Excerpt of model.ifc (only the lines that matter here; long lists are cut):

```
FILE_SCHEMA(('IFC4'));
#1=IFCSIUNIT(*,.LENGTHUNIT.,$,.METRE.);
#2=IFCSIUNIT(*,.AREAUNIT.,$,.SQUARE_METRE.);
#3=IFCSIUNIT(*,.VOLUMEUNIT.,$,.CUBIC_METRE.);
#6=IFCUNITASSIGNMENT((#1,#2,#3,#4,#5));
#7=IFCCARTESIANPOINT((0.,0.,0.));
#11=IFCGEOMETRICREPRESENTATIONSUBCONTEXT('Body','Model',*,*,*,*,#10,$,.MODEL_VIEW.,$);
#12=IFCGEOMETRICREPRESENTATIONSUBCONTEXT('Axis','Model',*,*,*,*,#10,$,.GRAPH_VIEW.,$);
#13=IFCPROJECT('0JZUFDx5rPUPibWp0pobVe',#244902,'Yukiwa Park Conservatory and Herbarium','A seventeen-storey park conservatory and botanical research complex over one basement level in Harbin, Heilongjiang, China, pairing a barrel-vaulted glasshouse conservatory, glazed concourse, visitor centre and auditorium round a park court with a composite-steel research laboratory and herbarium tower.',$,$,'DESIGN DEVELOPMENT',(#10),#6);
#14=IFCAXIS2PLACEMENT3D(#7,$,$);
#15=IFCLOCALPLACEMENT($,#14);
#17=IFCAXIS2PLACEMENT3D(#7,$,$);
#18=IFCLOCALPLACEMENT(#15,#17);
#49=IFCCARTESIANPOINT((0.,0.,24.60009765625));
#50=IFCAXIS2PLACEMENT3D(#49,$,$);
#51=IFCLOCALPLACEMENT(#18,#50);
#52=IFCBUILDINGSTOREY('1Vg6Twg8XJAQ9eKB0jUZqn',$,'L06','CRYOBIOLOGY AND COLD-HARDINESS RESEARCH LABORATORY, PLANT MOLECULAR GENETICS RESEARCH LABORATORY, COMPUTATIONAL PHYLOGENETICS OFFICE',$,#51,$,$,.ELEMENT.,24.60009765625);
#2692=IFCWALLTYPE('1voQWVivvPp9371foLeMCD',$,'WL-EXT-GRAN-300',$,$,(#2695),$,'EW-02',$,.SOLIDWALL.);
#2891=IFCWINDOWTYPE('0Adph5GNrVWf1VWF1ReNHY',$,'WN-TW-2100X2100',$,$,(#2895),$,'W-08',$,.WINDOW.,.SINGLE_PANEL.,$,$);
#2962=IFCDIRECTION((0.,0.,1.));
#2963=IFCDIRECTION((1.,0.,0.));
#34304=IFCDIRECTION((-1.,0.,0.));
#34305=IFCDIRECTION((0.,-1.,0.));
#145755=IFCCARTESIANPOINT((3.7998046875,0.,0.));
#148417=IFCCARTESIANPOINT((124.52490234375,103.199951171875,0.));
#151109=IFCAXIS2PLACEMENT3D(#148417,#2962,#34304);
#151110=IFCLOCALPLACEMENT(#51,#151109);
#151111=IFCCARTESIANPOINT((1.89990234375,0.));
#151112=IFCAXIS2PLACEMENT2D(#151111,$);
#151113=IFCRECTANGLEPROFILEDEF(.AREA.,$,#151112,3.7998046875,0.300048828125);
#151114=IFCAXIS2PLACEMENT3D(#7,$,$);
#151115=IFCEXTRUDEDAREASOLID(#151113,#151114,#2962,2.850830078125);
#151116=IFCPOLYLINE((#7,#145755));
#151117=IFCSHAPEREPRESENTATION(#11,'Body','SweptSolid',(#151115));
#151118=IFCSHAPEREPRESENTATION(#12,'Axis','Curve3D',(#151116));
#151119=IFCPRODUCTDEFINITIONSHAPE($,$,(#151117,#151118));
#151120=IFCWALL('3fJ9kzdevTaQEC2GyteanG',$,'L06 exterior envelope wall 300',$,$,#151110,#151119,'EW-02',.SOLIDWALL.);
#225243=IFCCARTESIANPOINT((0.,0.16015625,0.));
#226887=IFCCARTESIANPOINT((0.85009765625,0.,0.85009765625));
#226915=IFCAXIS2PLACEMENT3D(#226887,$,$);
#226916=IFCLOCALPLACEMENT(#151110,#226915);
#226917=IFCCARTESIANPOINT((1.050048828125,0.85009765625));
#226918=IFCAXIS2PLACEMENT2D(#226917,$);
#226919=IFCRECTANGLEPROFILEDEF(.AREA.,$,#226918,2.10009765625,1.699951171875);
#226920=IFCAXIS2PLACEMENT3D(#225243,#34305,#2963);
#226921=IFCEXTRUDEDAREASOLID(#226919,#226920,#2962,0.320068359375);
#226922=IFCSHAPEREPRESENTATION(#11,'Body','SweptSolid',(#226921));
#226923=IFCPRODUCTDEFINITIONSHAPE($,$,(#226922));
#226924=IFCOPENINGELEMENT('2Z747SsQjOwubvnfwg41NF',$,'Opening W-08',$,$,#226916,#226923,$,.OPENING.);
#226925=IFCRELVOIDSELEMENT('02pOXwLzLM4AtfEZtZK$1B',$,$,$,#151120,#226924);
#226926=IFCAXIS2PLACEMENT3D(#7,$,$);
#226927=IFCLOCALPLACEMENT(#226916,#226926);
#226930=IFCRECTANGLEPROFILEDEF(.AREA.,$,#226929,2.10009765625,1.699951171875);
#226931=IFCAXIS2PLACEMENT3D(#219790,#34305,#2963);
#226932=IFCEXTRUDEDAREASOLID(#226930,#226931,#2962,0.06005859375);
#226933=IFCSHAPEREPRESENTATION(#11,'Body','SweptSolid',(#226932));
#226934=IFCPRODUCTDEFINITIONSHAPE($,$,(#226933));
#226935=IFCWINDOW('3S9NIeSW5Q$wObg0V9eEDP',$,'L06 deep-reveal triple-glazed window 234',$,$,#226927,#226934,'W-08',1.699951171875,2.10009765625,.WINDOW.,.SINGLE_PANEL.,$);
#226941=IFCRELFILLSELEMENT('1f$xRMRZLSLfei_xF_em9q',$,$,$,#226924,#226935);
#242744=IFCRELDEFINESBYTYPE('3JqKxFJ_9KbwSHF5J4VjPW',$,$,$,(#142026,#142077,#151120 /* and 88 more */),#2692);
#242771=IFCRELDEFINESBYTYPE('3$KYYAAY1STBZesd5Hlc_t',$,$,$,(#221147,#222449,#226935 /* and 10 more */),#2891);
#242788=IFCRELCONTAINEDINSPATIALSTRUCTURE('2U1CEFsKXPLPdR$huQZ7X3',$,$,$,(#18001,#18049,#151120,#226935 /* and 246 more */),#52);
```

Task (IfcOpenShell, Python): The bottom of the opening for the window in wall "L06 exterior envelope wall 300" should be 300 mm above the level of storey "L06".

```python
import numpy as np
import ifcopenshell
import ifcopenshell.api.geometry
import ifcopenshell.geom
import ifcopenshell.util.element
import ifcopenshell.util.placement
import ifcopenshell.util.shape
import ifcopenshell.util.unit

model = ifcopenshell.open("model.ifc")
unit_scale = ifcopenshell.util.unit.calculate_unit_scale(model)

window = model.by_guid("3S9NIeSW5Q$wObg0V9eEDP")
opening = window.FillsVoids[0].RelatingOpeningElement
storey = ifcopenshell.util.element.get_container(window, ifc_class="IfcBuildingStorey")
level = ifcopenshell.util.placement.get_local_placement(storey.ObjectPlacement)[2, 3]

# The opening's origin need not be at the sill, so measure its lowest point.
shape = ifcopenshell.geom.create_shape(ifcopenshell.geom.settings(), opening)
bottom = ifcopenshell.util.shape.get_shape_bottom_elevation(shape, shape.geometry) / unit_scale
dz = level + 0.3 / unit_scale - bottom

shift = np.array([0.0, 0.0, dz])
# The window is placed relative to its opening, so it follows when the opening moves.
matrix = ifcopenshell.util.placement.get_local_placement(opening.ObjectPlacement)
matrix[:3, 3] += shift
ifcopenshell.api.geometry.edit_object_placement(
    model, product=opening, matrix=matrix, is_si=False, should_transform_children=True
)

print(f"moved by {dz * unit_scale:+.3f} m")

model.write("model_v2.ifc")
```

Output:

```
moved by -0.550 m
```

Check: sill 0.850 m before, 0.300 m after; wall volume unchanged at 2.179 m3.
